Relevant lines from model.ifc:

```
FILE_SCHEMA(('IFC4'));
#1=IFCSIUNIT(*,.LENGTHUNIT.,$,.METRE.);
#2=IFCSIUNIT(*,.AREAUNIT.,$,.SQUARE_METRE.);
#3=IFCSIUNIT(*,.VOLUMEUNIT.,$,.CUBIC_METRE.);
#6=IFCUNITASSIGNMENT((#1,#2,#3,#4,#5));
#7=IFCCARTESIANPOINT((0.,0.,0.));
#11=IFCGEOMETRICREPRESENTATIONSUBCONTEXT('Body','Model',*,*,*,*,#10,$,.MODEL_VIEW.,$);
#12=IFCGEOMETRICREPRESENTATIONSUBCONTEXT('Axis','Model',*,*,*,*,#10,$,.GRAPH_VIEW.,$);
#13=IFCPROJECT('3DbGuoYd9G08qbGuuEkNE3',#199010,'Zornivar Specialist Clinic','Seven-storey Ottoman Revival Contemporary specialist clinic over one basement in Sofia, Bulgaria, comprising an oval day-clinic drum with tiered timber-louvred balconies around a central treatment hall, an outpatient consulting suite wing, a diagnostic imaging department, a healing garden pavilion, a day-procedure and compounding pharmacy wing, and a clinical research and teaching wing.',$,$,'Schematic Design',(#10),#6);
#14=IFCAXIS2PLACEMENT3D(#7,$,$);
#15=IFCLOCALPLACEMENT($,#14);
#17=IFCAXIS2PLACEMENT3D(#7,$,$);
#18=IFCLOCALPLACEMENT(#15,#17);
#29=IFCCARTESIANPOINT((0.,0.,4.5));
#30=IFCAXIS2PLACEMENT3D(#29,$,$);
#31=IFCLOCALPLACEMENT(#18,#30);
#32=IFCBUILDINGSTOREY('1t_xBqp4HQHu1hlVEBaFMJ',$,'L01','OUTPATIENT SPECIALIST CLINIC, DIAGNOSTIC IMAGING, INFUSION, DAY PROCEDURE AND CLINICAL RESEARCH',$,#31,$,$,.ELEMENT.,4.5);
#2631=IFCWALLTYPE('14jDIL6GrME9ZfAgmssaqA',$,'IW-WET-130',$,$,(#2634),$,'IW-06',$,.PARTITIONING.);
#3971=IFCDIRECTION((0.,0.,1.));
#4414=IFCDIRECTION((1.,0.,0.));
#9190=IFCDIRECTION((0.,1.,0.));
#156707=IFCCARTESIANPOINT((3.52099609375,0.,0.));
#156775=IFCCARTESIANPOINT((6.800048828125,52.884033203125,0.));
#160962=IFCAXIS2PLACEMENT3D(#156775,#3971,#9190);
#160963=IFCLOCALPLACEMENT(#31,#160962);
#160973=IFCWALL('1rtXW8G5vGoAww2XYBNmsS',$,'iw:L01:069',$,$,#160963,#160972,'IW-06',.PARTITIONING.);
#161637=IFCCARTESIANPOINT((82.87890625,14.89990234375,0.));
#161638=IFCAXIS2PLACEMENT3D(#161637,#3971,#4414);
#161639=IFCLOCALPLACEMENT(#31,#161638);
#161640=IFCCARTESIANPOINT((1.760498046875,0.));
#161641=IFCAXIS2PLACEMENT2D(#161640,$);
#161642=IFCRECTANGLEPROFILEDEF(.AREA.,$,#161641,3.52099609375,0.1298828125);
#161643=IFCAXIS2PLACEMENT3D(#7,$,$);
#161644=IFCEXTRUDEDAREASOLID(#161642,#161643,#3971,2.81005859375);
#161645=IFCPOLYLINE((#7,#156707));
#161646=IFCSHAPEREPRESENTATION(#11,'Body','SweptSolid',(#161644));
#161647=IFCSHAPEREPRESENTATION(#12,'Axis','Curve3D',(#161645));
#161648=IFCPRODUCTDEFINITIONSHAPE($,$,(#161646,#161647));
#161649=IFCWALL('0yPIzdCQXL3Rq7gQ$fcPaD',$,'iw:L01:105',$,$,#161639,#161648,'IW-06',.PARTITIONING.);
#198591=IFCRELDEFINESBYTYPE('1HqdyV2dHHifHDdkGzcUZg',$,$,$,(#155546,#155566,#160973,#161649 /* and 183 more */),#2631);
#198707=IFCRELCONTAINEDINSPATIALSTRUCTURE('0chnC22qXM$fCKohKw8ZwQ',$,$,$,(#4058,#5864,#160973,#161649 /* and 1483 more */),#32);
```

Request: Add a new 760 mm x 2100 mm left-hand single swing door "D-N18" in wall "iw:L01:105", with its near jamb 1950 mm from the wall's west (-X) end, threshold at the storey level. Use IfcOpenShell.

```python
import numpy as np
import ifcopenshell
import ifcopenshell.api.feature
import ifcopenshell.api.geometry
import ifcopenshell.api.root
import ifcopenshell.api.spatial
import ifcopenshell.geom
import ifcopenshell.util.element
import ifcopenshell.util.placement
import ifcopenshell.util.representation
import ifcopenshell.util.shape
import ifcopenshell.util.unit

model = ifcopenshell.open("model.ifc")
unit_scale = ifcopenshell.util.unit.calculate_unit_scale(model)
settings = ifcopenshell.geom.settings()


def volume(element):
    """Net volume in cubic metres, openings subtracted."""
    shape = ifcopenshell.geom.create_shape(settings, element)
    return ifcopenshell.util.shape.get_volume(shape.geometry)


wall = model.by_guid("0yPIzdCQXL3Rq7gQ$fcPaD")
storey = ifcopenshell.util.element.get_container(wall, ifc_class="IfcBuildingStorey")
context = ifcopenshell.util.representation.get_context(model, "Model", "Body", "MODEL_VIEW")
before = volume(wall)

width, height, from_end, sill = 0.76, 2.1, 1.95, 0.0  # metres

# The wall runs along its own X axis, and the end named is its -X end.
wall_shape = ifcopenshell.geom.create_shape(settings, wall)
x, y, z = ifcopenshell.util.shape.get_vertices(wall_shape.geometry).T
start = x.min() + from_end
face, thickness = float(y.min()), float(y.max() - y.min())
wall_matrix = ifcopenshell.util.placement.get_local_placement(wall.ObjectPlacement)
level = ifcopenshell.util.placement.get_local_placement(storey.ObjectPlacement)[2, 3]


def in_wall(x, y):
    """Placement at x, y metres in the wall's axes, at sill height."""
    matrix = wall_matrix.copy()
    matrix[:, 3] = wall_matrix @ np.array([x / unit_scale, y / unit_scale, 0.0, 1.0])
    matrix[2, 3] = level + sill / unit_scale
    return matrix


# Opening: a box that overshoots both wall faces by 50 mm.
opening = ifcopenshell.api.root.create_entity(model, ifc_class="IfcOpeningElement", predefined_type="OPENING")
box = ifcopenshell.api.geometry.add_wall_representation(
    model, context=context, length=width, height=height, thickness=thickness + 0.1
)
ifcopenshell.api.geometry.assign_representation(model, product=opening, representation=box)
ifcopenshell.api.geometry.edit_object_placement(model, product=opening, matrix=in_wall(start, face - 0.05), is_si=False)
ifcopenshell.api.feature.add_feature(model, feature=opening, element=wall)

door = ifcopenshell.api.root.create_entity(model, ifc_class="IfcDoor", name="D-N18", predefined_type="DOOR")
door.OverallWidth, door.OverallHeight = width / unit_scale, height / unit_scale
door.OperationType = "SINGLE_SWING_LEFT"
body = ifcopenshell.api.geometry.add_door_representation(
    model,
    context=context,
    overall_width=door.OverallWidth,
    overall_height=door.OverallHeight,
    operation_type="SINGLE_SWING_LEFT",
    lining_properties={"LiningDepth": thickness / unit_scale, "ThresholdDepth": thickness / unit_scale},
)
ifcopenshell.api.geometry.assign_representation(model, product=door, representation=body)
ifcopenshell.api.spatial.assign_container(model, products=[door], relating_structure=storey)
ifcopenshell.api.feature.add_filling(model, opening=opening, element=door)

# The lining spans the wall, so the door starts at the wall face.
ifcopenshell.api.geometry.edit_object_placement(model, product=door, matrix=in_wall(start, face), is_si=False)

after = volume(wall)

print(f"wall volume {before:.3f} -> {after:.3f} m3")

model.write("model_edited.ifc")
```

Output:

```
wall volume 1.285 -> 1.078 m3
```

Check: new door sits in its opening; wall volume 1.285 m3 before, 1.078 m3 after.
